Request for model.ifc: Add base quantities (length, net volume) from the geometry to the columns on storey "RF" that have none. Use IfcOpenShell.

First a look at what the model holds.

```python
import ifcopenshell
import ifcopenshell.util.element
import ifcopenshell.util.unit

model = ifcopenshell.open("model.ifc")
print(model.schema)
for unit_type in ("LENGTHUNIT", "AREAUNIT", "VOLUMEUNIT"):
    print(unit_type, ifcopenshell.util.unit.calculate_unit_scale(model, unit_type))
storey = next(s for s in model.by_type("IfcBuildingStorey") if s.Name == "RF")
columns = [e for e in ifcopenshell.util.element.get_decomposition(storey) if e.is_a("IfcColumn")]
for e in sorted(columns, key=lambda e: e.id()):
    print(e.id(), e.is_a(), e.Name, list(ifcopenshell.util.element.get_psets(e, qtos_only=True)), sep=" | ")
```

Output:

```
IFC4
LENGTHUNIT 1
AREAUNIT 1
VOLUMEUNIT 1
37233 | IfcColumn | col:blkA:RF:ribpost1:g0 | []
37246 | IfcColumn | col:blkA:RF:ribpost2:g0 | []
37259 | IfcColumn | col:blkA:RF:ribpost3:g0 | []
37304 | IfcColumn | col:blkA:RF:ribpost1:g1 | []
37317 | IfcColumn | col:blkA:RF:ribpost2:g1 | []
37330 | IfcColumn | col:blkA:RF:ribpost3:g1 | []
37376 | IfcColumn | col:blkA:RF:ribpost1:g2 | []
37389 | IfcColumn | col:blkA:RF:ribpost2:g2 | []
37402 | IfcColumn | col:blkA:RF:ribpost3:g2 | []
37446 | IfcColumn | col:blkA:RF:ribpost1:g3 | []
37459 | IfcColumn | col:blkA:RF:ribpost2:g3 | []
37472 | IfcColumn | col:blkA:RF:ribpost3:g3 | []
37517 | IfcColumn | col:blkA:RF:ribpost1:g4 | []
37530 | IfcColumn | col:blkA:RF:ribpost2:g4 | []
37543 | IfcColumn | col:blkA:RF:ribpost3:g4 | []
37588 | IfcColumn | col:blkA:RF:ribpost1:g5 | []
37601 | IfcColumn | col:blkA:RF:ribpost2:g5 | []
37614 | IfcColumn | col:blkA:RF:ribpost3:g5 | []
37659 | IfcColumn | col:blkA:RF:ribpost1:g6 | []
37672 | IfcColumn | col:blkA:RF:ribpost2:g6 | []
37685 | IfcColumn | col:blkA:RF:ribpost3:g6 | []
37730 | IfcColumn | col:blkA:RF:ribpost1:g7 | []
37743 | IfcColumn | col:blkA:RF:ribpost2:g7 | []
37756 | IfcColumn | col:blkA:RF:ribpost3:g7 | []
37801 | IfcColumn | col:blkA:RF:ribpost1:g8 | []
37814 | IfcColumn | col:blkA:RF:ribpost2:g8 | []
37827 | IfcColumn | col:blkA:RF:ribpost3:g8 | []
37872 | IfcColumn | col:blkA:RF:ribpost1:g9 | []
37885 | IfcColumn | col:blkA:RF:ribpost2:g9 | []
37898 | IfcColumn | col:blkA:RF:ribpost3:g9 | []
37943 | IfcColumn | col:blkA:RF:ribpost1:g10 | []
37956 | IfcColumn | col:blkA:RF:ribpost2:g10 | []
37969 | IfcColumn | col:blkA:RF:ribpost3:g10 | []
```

```python
import ifcopenshell
import ifcopenshell.api.pset
import ifcopenshell.geom
import ifcopenshell.util.element
import ifcopenshell.util.shape
import ifcopenshell.util.unit

model = ifcopenshell.open("model.ifc")
unit_scale = ifcopenshell.util.unit.calculate_unit_scale(model)
volume_scale = ifcopenshell.util.unit.calculate_unit_scale(model, "VOLUMEUNIT")
settings = ifcopenshell.geom.settings()

storey = next(s for s in model.by_type("IfcBuildingStorey") if s.Name == "RF")
columns = [e for e in ifcopenshell.util.element.get_decomposition(storey) if e.is_a("IfcColumn")]

for e in sorted(columns, key=lambda e: e.id()):
    if ifcopenshell.util.element.get_psets(e, qtos_only=True, should_inherit=False):
        continue
    # Geometry comes back in metres, in the element's own axes.
    shape = ifcopenshell.geom.create_shape(settings, e)
    values = {
        "Length": ifcopenshell.util.shape.get_z(shape.geometry) / unit_scale,
        "NetVolume": ifcopenshell.util.shape.get_volume(shape.geometry) / volume_scale,
    }
    qto = ifcopenshell.api.pset.add_qto(model, product=e, name="Qto_ColumnBaseQuantities")
    ifcopenshell.api.pset.edit_qto(model, qto=qto, properties=values)
    print(e.id(), {k: round(v, 3) for k, v in values.items()})

model.write("model-out.ifc")
```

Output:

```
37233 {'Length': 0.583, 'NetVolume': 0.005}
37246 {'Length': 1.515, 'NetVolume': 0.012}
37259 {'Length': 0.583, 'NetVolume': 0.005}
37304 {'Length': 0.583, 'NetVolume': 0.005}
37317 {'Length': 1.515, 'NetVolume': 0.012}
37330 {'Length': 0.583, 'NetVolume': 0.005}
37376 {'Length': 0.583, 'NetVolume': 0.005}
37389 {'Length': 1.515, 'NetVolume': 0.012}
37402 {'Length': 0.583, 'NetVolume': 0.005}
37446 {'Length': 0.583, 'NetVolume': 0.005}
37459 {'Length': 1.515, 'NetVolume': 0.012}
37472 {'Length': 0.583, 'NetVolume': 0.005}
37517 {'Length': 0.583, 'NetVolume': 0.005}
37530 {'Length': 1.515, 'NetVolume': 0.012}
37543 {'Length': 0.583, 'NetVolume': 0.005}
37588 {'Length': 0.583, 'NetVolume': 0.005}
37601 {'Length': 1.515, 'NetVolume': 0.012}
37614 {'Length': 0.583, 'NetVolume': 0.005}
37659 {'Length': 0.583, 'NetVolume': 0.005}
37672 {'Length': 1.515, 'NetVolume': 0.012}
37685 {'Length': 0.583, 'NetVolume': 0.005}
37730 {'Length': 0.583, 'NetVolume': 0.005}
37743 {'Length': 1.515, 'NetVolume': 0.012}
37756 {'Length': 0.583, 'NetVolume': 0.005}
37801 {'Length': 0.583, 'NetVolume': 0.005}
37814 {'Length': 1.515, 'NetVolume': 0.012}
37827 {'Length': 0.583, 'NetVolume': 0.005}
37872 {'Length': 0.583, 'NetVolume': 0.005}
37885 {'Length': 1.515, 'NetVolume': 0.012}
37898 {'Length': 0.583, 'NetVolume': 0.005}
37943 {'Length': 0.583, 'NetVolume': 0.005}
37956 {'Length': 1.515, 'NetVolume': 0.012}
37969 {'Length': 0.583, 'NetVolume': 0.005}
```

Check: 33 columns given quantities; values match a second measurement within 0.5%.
